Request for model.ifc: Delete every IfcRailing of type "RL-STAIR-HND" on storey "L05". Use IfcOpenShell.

First a look at what the model holds.

```python
import ifcopenshell
import ifcopenshell.util.element

model = ifcopenshell.open("model.ifc")
print(model.schema)
storey = next(s for s in model.by_type("IfcBuildingStorey") if s.Name == "L05")
railings = [e for e in ifcopenshell.util.element.get_decomposition(storey) if e.is_a("IfcRailing")]
seen = {}
for e in railings:
    element_type = ifcopenshell.util.element.get_type(e)
    name = element_type.Name if element_type not in (None, e) else None
    seen[name] = seen.get(name, 0) + 1
for name, count in sorted(seen.items(), key=str):
    print(count, "x", name)
```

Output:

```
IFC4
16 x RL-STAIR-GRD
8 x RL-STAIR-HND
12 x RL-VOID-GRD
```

```python
import ifcopenshell
import ifcopenshell.api.root
import ifcopenshell.util.element

model = ifcopenshell.open("model.ifc")

storey = next(s for s in model.by_type("IfcBuildingStorey") if s.Name == "L05")
railings = [e for e in ifcopenshell.util.element.get_decomposition(storey) if e.is_a("IfcRailing")]
targets = [e for e in railings if (t := ifcopenshell.util.element.get_type(e)) not in (None, e) and t.Name == "RL-STAIR-HND"]

for e in targets:
    ifcopenshell.api.root.remove_product(model, product=e)
print(len(targets), "removed")

model.write("model_rev.ifc")
```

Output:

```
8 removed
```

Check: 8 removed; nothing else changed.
